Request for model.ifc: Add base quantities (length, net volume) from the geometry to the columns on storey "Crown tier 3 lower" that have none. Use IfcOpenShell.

First a look at what the model holds.

```python
import ifcopenshell
import ifcopenshell.util.element
import ifcopenshell.util.unit

model = ifcopenshell.open("model.ifc")
print(model.schema)
for unit_type in ("LENGTHUNIT", "AREAUNIT", "VOLUMEUNIT"):
    print(unit_type, ifcopenshell.util.unit.calculate_unit_scale(model, unit_type))
storey = next(s for s in model.by_type("IfcBuildingStorey") if s.Name == "Crown tier 3 lower")
columns = [e for e in ifcopenshell.util.element.get_decomposition(storey) if e.is_a("IfcColumn")]
for e in sorted(columns, key=lambda e: e.id()):
    print(e.id(), e.is_a(), e.Name, list(ifcopenshell.util.element.get_psets(e, qtos_only=True)), sep=" | ")
```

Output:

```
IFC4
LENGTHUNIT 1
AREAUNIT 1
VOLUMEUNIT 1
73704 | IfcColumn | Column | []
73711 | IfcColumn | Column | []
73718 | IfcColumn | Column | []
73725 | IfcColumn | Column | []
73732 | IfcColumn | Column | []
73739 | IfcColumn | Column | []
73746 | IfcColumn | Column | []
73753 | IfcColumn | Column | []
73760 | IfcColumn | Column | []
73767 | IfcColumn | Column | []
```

```python
import ifcopenshell
import ifcopenshell.api.pset
import ifcopenshell.geom
import ifcopenshell.util.element
import ifcopenshell.util.shape
import ifcopenshell.util.unit

model = ifcopenshell.open("model.ifc")
unit_scale = ifcopenshell.util.unit.calculate_unit_scale(model)
volume_scale = ifcopenshell.util.unit.calculate_unit_scale(model, "VOLUMEUNIT")
settings = ifcopenshell.geom.settings()

storey = next(s for s in model.by_type("IfcBuildingStorey") if s.Name == "Crown tier 3 lower")
columns = [e for e in ifcopenshell.util.element.get_decomposition(storey) if e.is_a("IfcColumn")]

for e in sorted(columns, key=lambda e: e.id()):
    if ifcopenshell.util.element.get_psets(e, qtos_only=True, should_inherit=False):
        continue
    # Geometry comes back in metres, in the element's own axes.
    shape = ifcopenshell.geom.create_shape(settings, e)
    values = {
        "Length": ifcopenshell.util.shape.get_z(shape.geometry) / unit_scale,
        "NetVolume": ifcopenshell.util.shape.get_volume(shape.geometry) / volume_scale,
    }
    qto = ifcopenshell.api.pset.add_qto(model, product=e, name="Qto_ColumnBaseQuantities")
    ifcopenshell.api.pset.edit_qto(model, qto=qto, properties=values)
    print(e.id(), {k: round(v, 3) for k, v in values.items()})

model.write("model_edited.ifc")
```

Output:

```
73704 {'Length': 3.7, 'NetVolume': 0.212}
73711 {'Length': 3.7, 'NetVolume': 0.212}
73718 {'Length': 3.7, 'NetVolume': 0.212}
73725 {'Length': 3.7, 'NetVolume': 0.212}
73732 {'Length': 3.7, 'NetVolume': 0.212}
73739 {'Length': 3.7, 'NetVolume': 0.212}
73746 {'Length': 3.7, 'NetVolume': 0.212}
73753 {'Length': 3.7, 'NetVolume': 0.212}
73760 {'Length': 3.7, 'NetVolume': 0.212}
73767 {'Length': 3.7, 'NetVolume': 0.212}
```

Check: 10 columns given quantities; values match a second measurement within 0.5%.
